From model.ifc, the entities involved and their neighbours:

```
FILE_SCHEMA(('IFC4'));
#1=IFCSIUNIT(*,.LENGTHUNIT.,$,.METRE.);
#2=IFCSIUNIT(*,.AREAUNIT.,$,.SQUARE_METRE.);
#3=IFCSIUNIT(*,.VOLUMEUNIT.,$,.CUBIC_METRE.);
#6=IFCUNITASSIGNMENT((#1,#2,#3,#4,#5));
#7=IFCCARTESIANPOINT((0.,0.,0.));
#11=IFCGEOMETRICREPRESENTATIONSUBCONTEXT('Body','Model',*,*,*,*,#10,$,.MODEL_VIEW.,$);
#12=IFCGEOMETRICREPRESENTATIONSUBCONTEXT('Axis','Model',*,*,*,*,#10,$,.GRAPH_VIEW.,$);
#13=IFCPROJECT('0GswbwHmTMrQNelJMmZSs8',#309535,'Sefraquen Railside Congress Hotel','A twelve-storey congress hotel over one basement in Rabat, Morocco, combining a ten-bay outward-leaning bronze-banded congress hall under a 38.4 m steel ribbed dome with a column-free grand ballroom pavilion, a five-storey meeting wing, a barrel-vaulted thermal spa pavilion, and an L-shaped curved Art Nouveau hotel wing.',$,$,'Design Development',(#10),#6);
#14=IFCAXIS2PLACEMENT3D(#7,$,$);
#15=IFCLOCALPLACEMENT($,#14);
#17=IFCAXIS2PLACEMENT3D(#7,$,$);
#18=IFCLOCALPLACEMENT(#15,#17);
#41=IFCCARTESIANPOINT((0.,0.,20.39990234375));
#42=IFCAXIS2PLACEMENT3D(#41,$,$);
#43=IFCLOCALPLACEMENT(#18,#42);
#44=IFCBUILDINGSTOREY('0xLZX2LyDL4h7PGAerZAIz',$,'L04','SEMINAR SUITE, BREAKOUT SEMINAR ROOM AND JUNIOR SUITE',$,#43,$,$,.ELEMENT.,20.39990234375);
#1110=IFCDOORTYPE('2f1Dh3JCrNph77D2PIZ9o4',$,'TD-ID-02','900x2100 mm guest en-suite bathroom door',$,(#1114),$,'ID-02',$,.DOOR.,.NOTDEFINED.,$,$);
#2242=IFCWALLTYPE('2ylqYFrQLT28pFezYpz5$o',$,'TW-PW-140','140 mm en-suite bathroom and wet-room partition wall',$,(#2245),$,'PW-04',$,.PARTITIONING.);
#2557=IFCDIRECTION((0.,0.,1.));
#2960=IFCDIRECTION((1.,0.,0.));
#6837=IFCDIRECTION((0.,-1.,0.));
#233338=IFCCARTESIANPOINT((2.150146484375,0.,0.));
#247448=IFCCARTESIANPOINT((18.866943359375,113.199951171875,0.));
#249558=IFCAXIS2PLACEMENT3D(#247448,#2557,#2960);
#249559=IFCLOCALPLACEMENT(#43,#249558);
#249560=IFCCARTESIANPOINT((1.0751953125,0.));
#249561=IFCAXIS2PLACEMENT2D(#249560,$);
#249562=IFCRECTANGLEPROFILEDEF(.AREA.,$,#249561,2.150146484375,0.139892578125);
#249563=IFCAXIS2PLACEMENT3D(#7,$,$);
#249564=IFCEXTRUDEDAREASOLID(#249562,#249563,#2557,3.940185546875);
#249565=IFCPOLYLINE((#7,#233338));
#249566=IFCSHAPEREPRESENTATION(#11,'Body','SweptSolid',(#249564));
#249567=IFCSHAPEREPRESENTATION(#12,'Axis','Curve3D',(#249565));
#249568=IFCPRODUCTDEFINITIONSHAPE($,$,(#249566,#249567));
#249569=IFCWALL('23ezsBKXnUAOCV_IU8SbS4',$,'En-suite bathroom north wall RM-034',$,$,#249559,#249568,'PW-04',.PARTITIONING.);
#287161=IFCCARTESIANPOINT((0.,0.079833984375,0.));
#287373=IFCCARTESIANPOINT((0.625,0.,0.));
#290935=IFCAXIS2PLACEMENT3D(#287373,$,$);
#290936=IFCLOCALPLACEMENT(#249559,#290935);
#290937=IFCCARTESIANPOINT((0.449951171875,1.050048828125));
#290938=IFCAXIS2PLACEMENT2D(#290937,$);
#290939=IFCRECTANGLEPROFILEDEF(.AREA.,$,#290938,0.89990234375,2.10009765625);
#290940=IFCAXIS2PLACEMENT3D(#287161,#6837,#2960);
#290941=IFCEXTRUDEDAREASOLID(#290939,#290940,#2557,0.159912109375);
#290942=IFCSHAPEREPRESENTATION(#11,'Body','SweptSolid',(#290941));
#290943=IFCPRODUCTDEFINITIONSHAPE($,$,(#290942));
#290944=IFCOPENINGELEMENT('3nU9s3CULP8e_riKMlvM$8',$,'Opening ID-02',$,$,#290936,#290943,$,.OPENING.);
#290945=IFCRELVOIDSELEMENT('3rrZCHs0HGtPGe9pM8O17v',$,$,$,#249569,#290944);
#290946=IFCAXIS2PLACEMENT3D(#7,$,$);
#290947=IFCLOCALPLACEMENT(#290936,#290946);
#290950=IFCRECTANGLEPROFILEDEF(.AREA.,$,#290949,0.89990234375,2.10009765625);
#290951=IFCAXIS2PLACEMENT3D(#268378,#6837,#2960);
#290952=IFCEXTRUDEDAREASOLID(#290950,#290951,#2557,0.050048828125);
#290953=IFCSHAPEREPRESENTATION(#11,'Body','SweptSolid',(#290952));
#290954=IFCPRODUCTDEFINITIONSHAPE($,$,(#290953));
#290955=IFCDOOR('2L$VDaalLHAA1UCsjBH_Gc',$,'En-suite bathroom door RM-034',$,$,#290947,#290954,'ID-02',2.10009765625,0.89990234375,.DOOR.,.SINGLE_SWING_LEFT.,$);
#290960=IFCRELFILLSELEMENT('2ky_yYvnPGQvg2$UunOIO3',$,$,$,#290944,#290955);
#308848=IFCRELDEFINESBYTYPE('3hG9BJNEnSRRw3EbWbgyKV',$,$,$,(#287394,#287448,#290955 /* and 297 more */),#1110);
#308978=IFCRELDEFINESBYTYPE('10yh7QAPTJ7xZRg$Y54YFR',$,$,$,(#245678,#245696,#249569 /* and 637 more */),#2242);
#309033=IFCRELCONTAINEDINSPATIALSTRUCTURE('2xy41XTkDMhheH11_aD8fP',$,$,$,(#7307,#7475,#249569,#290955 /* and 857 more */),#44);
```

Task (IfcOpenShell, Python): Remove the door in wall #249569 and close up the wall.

```python
import ifcopenshell
import ifcopenshell.api.feature
import ifcopenshell.api.root
import ifcopenshell.geom
import ifcopenshell.util.shape

model = ifcopenshell.open("model.ifc")
settings = ifcopenshell.geom.settings()


def volume(element):
    """Net volume in cubic metres, openings subtracted."""
    shape = ifcopenshell.geom.create_shape(settings, element)
    return ifcopenshell.util.shape.get_volume(shape.geometry)


door = model.by_id(290955)
opening = door.FillsVoids[0].RelatingOpeningElement
wall = opening.VoidsElements[0].RelatingBuildingElement
before = volume(wall)

ifcopenshell.api.root.remove_product(model, product=door)
ifcopenshell.api.feature.remove_feature(model, feature=opening)

after = volume(wall)

print(f"wall volume {before:.3f} -> {after:.3f} m3")

model.write("model_edited.ifc")
```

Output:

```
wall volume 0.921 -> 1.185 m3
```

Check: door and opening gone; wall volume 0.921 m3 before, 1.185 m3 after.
